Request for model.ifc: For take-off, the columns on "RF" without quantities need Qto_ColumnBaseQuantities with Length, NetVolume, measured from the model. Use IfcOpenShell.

First a look at what the model holds.

```python
import ifcopenshell
import ifcopenshell.util.element
import ifcopenshell.util.unit

model = ifcopenshell.open("model.ifc")
print(model.schema)
for unit_type in ("LENGTHUNIT", "AREAUNIT", "VOLUMEUNIT"):
    print(unit_type, ifcopenshell.util.unit.calculate_unit_scale(model, unit_type))
storey = next(s for s in model.by_type("IfcBuildingStorey") if s.Name == "RF")
columns = [e for e in ifcopenshell.util.element.get_decomposition(storey) if e.is_a("IfcColumn")]
for e in sorted(columns, key=lambda e: e.id()):
    print(e.id(), e.is_a(), e.Name, list(ifcopenshell.util.element.get_psets(e, qtos_only=True)), sep=" | ")
```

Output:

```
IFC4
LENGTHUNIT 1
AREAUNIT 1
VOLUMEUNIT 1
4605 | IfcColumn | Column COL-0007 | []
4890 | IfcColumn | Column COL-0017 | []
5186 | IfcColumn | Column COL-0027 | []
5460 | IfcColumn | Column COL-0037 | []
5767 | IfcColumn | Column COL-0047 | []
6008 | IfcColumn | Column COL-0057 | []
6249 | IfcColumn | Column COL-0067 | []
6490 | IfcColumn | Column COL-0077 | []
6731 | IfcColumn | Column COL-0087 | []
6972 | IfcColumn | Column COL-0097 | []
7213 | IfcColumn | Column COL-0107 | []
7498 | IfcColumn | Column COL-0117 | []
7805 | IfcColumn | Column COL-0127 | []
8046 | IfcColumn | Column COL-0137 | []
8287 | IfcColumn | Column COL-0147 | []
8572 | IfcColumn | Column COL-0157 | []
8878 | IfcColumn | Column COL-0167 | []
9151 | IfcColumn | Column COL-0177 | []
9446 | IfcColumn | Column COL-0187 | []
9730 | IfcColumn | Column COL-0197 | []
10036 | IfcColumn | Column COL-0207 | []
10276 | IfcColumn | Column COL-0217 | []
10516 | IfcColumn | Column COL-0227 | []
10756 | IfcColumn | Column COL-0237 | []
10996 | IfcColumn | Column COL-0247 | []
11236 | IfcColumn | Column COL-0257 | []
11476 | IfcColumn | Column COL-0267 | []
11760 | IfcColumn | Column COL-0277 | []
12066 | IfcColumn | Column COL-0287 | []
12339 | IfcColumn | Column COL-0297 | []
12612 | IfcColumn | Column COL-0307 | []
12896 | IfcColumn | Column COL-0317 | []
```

```python
import ifcopenshell
import ifcopenshell.api.pset
import ifcopenshell.geom
import ifcopenshell.util.element
import ifcopenshell.util.shape
import ifcopenshell.util.unit

model = ifcopenshell.open("model.ifc")
unit_scale = ifcopenshell.util.unit.calculate_unit_scale(model)
volume_scale = ifcopenshell.util.unit.calculate_unit_scale(model, "VOLUMEUNIT")
settings = ifcopenshell.geom.settings()

storey = next(s for s in model.by_type("IfcBuildingStorey") if s.Name == "RF")
columns = [e for e in ifcopenshell.util.element.get_decomposition(storey) if e.is_a("IfcColumn")]

for e in sorted(columns, key=lambda e: e.id()):
    if ifcopenshell.util.element.get_psets(e, qtos_only=True, should_inherit=False):
        continue
    # Geometry comes back in metres, in the element's own axes.
    shape = ifcopenshell.geom.create_shape(settings, e)
    values = {
        "Length": ifcopenshell.util.shape.get_z(shape.geometry) / unit_scale,
        "NetVolume": ifcopenshell.util.shape.get_volume(shape.geometry) / volume_scale,
    }
    qto = ifcopenshell.api.pset.add_qto(model, product=e, name="Qto_ColumnBaseQuantities")
    ifcopenshell.api.pset.edit_qto(model, qto=qto, properties=values)
    print(e.id(), {k: round(v, 3) for k, v in values.items()})

model.write("model_updated.ifc")
```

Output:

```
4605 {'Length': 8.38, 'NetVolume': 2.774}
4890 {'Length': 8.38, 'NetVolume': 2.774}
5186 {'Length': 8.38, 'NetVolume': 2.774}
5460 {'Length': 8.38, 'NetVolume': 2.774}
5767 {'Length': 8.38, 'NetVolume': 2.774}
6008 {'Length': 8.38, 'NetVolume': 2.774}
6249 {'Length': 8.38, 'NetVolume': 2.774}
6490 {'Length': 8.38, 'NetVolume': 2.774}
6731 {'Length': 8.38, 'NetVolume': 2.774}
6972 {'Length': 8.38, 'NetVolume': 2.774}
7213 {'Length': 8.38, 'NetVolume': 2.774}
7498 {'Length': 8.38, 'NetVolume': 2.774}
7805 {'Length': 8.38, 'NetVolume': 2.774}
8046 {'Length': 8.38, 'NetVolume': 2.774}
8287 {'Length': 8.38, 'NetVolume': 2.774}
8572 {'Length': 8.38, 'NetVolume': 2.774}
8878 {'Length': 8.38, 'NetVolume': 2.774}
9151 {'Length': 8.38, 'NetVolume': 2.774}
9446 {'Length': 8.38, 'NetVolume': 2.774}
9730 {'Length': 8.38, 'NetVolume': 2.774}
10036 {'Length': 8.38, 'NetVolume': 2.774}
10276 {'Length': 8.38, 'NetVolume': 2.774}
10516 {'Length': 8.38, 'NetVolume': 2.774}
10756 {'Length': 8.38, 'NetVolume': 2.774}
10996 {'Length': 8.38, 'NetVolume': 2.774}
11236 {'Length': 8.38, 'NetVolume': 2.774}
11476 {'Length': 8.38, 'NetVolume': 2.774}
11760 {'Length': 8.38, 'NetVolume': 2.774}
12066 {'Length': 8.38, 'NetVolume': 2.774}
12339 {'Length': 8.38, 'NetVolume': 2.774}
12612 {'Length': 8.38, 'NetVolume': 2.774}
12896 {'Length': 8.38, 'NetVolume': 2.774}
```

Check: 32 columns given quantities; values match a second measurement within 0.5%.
